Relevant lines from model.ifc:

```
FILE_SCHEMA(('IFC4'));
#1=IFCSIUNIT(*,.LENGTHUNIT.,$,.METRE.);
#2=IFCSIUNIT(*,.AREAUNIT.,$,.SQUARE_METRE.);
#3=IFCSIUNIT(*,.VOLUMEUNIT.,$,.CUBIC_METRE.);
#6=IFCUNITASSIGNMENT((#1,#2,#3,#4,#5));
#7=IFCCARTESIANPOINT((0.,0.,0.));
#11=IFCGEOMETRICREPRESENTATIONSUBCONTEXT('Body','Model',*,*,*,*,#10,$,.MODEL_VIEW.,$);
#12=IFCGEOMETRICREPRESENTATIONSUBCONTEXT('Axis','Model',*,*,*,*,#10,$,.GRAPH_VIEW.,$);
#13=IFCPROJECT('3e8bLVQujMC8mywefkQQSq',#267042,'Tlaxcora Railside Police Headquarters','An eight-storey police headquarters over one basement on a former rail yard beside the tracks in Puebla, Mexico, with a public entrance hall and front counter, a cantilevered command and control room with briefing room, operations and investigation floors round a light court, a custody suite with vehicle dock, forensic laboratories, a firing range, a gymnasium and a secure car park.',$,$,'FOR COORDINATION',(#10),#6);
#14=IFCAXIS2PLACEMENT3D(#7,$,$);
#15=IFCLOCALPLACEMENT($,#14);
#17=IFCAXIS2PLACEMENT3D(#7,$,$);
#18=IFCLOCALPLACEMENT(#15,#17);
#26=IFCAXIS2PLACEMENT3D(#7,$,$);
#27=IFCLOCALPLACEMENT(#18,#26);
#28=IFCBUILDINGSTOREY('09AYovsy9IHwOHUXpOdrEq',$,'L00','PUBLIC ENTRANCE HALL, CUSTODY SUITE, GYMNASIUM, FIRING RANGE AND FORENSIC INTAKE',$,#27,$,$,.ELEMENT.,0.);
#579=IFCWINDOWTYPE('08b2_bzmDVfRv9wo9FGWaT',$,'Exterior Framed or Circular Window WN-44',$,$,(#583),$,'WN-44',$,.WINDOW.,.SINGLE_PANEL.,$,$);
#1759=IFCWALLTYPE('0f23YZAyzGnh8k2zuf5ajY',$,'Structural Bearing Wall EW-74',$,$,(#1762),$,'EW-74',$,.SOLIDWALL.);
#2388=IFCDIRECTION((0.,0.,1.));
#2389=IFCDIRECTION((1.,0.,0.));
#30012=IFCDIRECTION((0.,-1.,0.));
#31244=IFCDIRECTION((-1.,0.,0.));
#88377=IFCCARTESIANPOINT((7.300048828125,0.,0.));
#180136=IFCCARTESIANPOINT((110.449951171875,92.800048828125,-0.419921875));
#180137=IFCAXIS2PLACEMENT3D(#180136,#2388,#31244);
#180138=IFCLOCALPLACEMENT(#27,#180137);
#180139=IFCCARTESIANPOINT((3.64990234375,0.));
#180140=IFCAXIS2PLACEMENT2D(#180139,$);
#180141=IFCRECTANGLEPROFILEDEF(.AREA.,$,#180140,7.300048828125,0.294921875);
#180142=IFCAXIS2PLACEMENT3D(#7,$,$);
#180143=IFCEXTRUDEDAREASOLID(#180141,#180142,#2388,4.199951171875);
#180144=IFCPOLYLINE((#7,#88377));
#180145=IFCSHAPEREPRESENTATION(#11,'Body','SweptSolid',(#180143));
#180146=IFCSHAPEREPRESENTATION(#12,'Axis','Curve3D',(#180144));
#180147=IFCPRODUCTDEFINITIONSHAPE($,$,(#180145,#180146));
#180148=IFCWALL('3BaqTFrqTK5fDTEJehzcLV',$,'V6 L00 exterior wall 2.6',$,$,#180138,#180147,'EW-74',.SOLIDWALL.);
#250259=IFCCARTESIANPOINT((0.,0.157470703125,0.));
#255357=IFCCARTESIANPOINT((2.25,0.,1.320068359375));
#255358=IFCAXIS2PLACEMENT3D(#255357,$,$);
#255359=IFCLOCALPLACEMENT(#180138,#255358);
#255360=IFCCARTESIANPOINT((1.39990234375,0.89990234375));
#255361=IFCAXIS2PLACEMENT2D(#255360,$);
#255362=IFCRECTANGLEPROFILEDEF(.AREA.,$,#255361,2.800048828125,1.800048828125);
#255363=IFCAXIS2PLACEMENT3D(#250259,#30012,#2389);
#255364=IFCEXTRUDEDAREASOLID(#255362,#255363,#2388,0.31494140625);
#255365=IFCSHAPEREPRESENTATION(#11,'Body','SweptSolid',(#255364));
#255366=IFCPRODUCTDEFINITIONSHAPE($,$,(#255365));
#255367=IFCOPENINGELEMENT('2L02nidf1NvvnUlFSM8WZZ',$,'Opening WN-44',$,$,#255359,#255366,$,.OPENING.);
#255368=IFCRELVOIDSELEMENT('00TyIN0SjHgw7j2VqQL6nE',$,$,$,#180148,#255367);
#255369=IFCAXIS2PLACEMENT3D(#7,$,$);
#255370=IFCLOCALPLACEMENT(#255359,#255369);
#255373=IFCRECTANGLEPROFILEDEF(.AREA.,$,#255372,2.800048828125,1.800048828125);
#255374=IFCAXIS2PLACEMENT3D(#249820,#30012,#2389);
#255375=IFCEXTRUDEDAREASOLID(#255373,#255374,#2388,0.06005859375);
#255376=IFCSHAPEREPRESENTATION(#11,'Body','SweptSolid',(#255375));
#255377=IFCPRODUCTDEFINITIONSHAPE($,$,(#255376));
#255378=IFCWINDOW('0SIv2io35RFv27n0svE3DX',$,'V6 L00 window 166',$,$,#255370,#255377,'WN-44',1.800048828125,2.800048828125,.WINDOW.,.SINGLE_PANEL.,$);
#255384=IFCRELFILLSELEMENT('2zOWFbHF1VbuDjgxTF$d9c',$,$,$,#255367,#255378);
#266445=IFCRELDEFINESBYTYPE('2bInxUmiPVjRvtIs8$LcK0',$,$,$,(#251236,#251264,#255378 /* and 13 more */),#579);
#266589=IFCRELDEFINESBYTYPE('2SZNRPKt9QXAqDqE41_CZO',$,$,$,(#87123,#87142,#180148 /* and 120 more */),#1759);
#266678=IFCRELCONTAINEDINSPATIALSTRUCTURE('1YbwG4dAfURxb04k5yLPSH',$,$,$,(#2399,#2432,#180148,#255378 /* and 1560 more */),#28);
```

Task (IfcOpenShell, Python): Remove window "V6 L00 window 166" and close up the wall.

```python
import ifcopenshell
import ifcopenshell.api.feature
import ifcopenshell.api.root
import ifcopenshell.geom
import ifcopenshell.util.shape

model = ifcopenshell.open("model.ifc")
settings = ifcopenshell.geom.settings()


def volume(element):
    """Net volume in cubic metres, openings subtracted."""
    shape = ifcopenshell.geom.create_shape(settings, element)
    return ifcopenshell.util.shape.get_volume(shape.geometry)


window = model.by_guid("0SIv2io35RFv27n0svE3DX")
opening = window.FillsVoids[0].RelatingOpeningElement
wall = opening.VoidsElements[0].RelatingBuildingElement
before = volume(wall)

ifcopenshell.api.root.remove_product(model, product=window)
ifcopenshell.api.feature.remove_feature(model, feature=opening)

after = volume(wall)

print(f"wall volume {before:.3f} -> {after:.3f} m3")

model.write("model_v2.ifc")
```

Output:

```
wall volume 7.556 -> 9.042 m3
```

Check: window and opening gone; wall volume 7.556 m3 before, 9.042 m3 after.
